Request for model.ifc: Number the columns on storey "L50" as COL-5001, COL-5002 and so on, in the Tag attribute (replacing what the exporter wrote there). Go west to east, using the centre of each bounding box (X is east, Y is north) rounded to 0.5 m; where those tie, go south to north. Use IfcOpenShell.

First a look at what the model holds.

```python
import ifcopenshell
import ifcopenshell.util.element
import ifcopenshell.util.placement

model = ifcopenshell.open("model.ifc")
print(model.schema)
storey = next(s for s in model.by_type("IfcBuildingStorey") if s.Name == "L50")
columns = [e for e in ifcopenshell.util.element.get_decomposition(storey) if e.is_a("IfcColumn")]
for e in sorted(columns, key=lambda e: e.id()):
    origin = ifcopenshell.util.placement.get_local_placement(e.ObjectPlacement)[:3, 3]
    print(e.id(), e.Tag, e.Name, origin.round(2) + 0.0, sep=" | ")
```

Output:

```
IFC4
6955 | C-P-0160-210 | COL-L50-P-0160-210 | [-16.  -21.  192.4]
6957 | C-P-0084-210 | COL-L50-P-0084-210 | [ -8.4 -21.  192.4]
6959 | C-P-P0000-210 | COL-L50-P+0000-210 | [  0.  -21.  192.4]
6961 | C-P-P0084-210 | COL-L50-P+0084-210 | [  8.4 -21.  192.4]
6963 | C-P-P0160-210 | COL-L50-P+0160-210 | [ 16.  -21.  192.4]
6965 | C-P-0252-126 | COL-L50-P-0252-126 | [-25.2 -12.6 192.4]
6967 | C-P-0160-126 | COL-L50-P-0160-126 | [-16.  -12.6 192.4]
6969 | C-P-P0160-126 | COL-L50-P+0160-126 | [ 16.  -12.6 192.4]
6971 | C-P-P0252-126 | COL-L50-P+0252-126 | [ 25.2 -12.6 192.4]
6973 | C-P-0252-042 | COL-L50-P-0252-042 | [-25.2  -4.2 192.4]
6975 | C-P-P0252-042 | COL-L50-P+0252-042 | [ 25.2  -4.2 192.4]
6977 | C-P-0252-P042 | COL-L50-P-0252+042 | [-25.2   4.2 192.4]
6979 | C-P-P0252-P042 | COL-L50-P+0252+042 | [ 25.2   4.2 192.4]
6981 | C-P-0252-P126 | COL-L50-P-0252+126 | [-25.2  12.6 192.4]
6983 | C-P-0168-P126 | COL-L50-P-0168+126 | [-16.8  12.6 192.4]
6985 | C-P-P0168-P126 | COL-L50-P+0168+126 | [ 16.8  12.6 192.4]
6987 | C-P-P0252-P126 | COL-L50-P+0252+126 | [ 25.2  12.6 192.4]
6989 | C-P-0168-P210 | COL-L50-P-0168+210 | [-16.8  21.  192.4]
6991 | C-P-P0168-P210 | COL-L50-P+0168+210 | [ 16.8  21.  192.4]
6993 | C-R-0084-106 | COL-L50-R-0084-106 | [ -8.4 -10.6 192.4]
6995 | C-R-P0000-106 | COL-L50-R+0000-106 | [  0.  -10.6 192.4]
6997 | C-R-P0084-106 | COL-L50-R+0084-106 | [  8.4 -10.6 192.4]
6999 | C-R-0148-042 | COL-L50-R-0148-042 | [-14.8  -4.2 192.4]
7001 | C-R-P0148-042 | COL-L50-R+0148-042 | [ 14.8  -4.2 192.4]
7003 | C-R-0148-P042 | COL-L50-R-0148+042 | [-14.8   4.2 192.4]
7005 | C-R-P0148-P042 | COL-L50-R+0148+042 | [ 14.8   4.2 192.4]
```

```python
import ifcopenshell
import ifcopenshell.geom
import ifcopenshell.util.element
import ifcopenshell.util.shape

model = ifcopenshell.open("model.ifc")
settings = ifcopenshell.geom.settings()
settings.set("use-world-coords", True)


def centre(element):
    shape = ifcopenshell.geom.create_shape(settings, element)
    return ifcopenshell.util.shape.get_bbox_centroid(shape.geometry)


storey = next(s for s in model.by_type("IfcBuildingStorey") if s.Name == "L50")
columns = [e for e in ifcopenshell.util.element.get_decomposition(storey) if e.is_a("IfcColumn")]

# Insertion points can sit at a corner or the storey origin, so sort by the geometry (in metres).
centres = {e: centre(e) for e in columns}
columns.sort(key=lambda e: (round(centres[e][0] / 0.5), centres[e][1]))

for i, e in enumerate(columns, start=1):
    number = f"COL-50{i:02d}"
    e.Tag = number
    print(e.id(), number)

model.write("model_v2.ifc")
```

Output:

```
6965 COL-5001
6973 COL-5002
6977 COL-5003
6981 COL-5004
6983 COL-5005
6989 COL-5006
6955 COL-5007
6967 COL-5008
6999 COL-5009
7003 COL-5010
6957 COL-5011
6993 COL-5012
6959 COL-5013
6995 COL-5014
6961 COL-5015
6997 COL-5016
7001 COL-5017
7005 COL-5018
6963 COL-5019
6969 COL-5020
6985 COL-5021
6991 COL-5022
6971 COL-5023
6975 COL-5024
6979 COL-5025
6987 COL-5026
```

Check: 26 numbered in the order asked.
